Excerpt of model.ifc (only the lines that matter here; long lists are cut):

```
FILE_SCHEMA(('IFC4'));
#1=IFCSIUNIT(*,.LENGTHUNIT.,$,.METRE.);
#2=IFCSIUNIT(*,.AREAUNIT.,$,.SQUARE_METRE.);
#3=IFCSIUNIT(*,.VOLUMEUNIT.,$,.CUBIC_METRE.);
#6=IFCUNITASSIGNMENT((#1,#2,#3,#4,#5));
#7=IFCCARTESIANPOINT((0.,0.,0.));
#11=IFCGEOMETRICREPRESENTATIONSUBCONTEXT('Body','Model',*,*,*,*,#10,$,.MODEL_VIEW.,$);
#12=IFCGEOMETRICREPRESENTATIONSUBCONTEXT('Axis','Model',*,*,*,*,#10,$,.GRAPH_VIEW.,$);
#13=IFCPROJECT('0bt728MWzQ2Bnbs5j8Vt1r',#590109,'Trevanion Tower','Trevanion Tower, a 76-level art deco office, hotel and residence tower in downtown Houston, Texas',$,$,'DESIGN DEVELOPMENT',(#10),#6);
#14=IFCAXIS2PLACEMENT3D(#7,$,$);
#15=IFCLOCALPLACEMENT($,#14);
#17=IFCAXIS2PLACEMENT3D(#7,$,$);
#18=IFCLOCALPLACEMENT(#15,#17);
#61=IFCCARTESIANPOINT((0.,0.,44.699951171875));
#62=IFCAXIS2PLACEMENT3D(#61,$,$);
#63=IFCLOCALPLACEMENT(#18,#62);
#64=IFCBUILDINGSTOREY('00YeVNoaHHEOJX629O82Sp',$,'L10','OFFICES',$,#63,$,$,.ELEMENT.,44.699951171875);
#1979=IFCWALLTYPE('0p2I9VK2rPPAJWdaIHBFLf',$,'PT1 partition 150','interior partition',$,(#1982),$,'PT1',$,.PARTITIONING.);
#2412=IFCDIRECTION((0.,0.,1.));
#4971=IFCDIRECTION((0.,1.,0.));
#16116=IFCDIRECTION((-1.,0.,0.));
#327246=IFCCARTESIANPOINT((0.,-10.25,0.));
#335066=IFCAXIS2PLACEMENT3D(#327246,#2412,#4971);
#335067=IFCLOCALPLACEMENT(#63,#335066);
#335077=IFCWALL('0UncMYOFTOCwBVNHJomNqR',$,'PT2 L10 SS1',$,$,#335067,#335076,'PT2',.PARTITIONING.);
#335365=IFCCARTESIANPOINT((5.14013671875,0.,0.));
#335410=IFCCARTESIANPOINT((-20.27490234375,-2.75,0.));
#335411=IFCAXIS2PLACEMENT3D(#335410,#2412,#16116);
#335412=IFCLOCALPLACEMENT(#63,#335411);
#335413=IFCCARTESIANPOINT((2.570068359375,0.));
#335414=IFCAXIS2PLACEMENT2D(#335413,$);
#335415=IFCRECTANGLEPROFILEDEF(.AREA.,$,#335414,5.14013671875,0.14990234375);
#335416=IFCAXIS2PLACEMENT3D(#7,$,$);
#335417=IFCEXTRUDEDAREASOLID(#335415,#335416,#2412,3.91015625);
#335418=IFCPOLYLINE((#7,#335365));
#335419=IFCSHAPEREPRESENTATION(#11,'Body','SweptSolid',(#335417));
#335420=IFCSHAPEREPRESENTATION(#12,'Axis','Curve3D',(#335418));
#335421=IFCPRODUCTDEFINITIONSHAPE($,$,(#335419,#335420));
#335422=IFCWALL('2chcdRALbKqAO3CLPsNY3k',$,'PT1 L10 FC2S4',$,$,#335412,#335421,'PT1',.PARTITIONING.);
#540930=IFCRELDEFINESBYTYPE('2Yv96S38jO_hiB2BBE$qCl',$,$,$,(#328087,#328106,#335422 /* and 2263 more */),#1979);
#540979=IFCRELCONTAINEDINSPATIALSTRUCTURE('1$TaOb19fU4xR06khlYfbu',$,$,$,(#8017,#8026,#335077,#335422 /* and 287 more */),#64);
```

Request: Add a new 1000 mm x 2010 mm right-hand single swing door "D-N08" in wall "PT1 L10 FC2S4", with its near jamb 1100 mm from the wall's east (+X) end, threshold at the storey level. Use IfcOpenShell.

```python
import numpy as np
import ifcopenshell
import ifcopenshell.api.feature
import ifcopenshell.api.geometry
import ifcopenshell.api.root
import ifcopenshell.api.spatial
import ifcopenshell.geom
import ifcopenshell.util.element
import ifcopenshell.util.placement
import ifcopenshell.util.representation
import ifcopenshell.util.shape
import ifcopenshell.util.unit

model = ifcopenshell.open("model.ifc")
unit_scale = ifcopenshell.util.unit.calculate_unit_scale(model)
settings = ifcopenshell.geom.settings()


def volume(element):
    """Net volume in cubic metres, openings subtracted."""
    shape = ifcopenshell.geom.create_shape(settings, element)
    return ifcopenshell.util.shape.get_volume(shape.geometry)


wall = model.by_guid("2chcdRALbKqAO3CLPsNY3k")
storey = ifcopenshell.util.element.get_container(wall, ifc_class="IfcBuildingStorey")
context = ifcopenshell.util.representation.get_context(model, "Model", "Body", "MODEL_VIEW")
before = volume(wall)

width, height, from_end, sill = 1, 2.01, 1.1, 0.0  # metres

# The wall runs along its own X axis, and the end named is its -X end.
wall_shape = ifcopenshell.geom.create_shape(settings, wall)
x, y, z = ifcopenshell.util.shape.get_vertices(wall_shape.geometry).T
start = x.min() + from_end
face, thickness = float(y.min()), float(y.max() - y.min())
wall_matrix = ifcopenshell.util.placement.get_local_placement(wall.ObjectPlacement)
level = ifcopenshell.util.placement.get_local_placement(storey.ObjectPlacement)[2, 3]


def in_wall(x, y):
    """Placement at x, y metres in the wall's axes, at sill height."""
    matrix = wall_matrix.copy()
    matrix[:, 3] = wall_matrix @ np.array([x / unit_scale, y / unit_scale, 0.0, 1.0])
    matrix[2, 3] = level + sill / unit_scale
    return matrix


# Opening: a box that overshoots both wall faces by 50 mm.
opening = ifcopenshell.api.root.create_entity(model, ifc_class="IfcOpeningElement", predefined_type="OPENING")
box = ifcopenshell.api.geometry.add_wall_representation(
    model, context=context, length=width, height=height, thickness=thickness + 0.1
)
ifcopenshell.api.geometry.assign_representation(model, product=opening, representation=box)
ifcopenshell.api.geometry.edit_object_placement(model, product=opening, matrix=in_wall(start, face - 0.05), is_si=False)
ifcopenshell.api.feature.add_feature(model, feature=opening, element=wall)

door = ifcopenshell.api.root.create_entity(model, ifc_class="IfcDoor", name="D-N08", predefined_type="DOOR")
door.OverallWidth, door.OverallHeight = width / unit_scale, height / unit_scale
door.OperationType = "SINGLE_SWING_RIGHT"
body = ifcopenshell.api.geometry.add_door_representation(
    model,
    context=context,
    overall_width=door.OverallWidth,
    overall_height=door.OverallHeight,
    operation_type="SINGLE_SWING_RIGHT",
    lining_properties={"LiningDepth": thickness / unit_scale, "ThresholdDepth": thickness / unit_scale},
)
ifcopenshell.api.geometry.assign_representation(model, product=door, representation=body)
ifcopenshell.api.spatial.assign_container(model, products=[door], relating_structure=storey)
ifcopenshell.api.feature.add_filling(model, opening=opening, element=door)

# The lining spans the wall, so the door starts at the wall face.
ifcopenshell.api.geometry.edit_object_placement(model, product=door, matrix=in_wall(start, face), is_si=False)

after = volume(wall)

print(f"wall volume {before:.3f} -> {after:.3f} m3")

model.write("model_v2.ifc")
```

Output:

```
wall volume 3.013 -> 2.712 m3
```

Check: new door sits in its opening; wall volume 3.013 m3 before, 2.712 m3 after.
